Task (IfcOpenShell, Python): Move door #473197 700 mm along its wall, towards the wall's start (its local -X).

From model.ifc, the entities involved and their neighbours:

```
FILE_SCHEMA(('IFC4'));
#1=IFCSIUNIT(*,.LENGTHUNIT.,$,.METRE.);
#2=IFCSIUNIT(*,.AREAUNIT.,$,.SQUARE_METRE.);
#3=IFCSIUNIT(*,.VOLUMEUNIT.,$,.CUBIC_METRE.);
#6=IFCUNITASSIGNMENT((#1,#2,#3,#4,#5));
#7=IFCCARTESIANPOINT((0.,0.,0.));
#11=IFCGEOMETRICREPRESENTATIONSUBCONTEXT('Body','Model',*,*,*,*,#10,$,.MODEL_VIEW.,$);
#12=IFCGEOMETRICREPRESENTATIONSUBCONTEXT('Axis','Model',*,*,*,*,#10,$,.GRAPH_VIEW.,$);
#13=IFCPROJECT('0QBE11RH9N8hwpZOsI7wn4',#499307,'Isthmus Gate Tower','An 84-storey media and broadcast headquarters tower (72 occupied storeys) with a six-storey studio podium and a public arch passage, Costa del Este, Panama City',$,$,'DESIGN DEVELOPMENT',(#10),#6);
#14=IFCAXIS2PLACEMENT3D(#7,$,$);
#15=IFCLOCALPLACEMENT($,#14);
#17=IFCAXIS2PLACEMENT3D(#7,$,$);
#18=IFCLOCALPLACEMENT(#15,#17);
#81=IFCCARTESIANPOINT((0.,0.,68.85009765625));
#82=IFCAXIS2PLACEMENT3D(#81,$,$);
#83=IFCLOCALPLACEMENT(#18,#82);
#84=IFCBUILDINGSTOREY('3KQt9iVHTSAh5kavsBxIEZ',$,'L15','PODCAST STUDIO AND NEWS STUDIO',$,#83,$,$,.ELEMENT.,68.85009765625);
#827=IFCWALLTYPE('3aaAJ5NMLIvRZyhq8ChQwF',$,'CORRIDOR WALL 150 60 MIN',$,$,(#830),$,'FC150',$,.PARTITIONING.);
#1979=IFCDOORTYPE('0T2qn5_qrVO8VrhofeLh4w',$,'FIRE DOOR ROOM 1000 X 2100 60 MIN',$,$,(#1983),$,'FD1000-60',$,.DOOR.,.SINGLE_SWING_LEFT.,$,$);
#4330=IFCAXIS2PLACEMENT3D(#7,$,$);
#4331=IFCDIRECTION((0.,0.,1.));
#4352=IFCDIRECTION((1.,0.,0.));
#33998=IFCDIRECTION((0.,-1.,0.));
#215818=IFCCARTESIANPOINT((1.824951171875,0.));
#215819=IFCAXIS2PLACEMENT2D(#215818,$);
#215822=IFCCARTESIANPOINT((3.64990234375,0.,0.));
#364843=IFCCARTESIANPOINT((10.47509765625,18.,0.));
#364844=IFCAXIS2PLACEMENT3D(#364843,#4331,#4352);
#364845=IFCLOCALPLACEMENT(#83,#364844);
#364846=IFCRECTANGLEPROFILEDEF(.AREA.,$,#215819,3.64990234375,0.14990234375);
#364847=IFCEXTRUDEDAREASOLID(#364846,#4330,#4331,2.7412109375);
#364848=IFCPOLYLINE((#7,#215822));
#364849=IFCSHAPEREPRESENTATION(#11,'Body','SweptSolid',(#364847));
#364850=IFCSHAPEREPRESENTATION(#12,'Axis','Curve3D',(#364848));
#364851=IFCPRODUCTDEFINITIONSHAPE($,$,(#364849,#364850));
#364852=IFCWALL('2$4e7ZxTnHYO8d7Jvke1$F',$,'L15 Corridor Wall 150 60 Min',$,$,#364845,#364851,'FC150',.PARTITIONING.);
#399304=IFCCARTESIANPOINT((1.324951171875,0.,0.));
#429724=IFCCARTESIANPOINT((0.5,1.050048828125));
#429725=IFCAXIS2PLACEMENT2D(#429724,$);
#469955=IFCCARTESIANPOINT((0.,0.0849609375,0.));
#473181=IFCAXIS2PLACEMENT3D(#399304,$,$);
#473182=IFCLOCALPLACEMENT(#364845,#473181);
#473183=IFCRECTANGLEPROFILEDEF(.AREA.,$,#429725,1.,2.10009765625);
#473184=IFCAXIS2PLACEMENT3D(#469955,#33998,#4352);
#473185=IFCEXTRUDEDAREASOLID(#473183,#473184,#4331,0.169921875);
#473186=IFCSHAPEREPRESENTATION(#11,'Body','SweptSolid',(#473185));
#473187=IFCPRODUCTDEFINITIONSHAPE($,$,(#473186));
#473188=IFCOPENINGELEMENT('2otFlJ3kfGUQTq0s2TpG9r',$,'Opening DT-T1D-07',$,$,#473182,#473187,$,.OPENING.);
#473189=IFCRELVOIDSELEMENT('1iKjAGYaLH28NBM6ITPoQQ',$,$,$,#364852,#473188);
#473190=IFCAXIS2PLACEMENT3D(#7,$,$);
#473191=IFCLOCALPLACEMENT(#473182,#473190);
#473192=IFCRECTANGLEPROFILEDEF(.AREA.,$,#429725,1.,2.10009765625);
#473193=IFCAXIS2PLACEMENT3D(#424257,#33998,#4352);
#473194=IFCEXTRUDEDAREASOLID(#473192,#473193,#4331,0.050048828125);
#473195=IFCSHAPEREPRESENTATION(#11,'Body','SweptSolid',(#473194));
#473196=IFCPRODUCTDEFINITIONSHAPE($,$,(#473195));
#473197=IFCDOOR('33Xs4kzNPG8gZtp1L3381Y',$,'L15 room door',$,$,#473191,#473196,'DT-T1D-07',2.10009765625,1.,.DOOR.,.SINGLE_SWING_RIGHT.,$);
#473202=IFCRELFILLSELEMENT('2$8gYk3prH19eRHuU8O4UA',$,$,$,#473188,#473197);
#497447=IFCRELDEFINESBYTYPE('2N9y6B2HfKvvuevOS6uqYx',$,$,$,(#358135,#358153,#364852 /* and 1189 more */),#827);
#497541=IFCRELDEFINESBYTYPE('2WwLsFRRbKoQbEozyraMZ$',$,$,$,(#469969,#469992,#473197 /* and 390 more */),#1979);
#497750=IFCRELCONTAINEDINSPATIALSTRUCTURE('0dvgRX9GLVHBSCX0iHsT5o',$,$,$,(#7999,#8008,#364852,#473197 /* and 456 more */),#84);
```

```python
import ifcopenshell
import ifcopenshell.api.geometry
import ifcopenshell.util.placement
import ifcopenshell.util.unit

model = ifcopenshell.open("model.ifc")
unit_scale = ifcopenshell.util.unit.calculate_unit_scale(model)

door = model.by_id(473197)
opening = door.FillsVoids[0].RelatingOpeningElement
wall = opening.VoidsElements[0].RelatingBuildingElement

wall_matrix = ifcopenshell.util.placement.get_local_placement(wall.ObjectPlacement)
shift = wall_matrix[:3, 0] * -0.7 / unit_scale
before = ifcopenshell.util.placement.get_local_placement(door.ObjectPlacement)[:3, 3].copy()

# The door is placed relative to its opening, so it follows when the opening moves.
matrix = ifcopenshell.util.placement.get_local_placement(opening.ObjectPlacement)
matrix[:3, 3] += shift
ifcopenshell.api.geometry.edit_object_placement(
    model, product=opening, matrix=matrix, is_si=False, should_transform_children=True
)

after = ifcopenshell.util.placement.get_local_placement(door.ObjectPlacement)[:3, 3]
print("door moved by", (after - before).round(3) + 0.0)

model.write("model_updated.ifc")
```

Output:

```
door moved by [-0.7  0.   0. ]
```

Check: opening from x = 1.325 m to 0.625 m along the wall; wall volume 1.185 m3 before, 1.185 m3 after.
